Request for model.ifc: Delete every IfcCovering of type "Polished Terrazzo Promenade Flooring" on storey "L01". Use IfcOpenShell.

First a look at what the model holds.

```python
import ifcopenshell
import ifcopenshell.util.element

model = ifcopenshell.open("model.ifc")
print(model.schema)
storey = next(s for s in model.by_type("IfcBuildingStorey") if s.Name == "L01")
coverings = [e for e in ifcopenshell.util.element.get_decomposition(storey) if e.is_a("IfcCovering")]
seen = {}
for e in coverings:
    element_type = ifcopenshell.util.element.get_type(e)
    name = element_type.Name if element_type not in (None, e) else None
    seen[name] = seen.get(name, 0) + 1
for name, count in sorted(seen.items(), key=str):
    print(count, "x", name)
```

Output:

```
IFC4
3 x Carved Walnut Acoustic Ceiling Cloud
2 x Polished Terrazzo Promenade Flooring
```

```python
import ifcopenshell
import ifcopenshell.api.root
import ifcopenshell.util.element

model = ifcopenshell.open("model.ifc")

storey = next(s for s in model.by_type("IfcBuildingStorey") if s.Name == "L01")
coverings = [e for e in ifcopenshell.util.element.get_decomposition(storey) if e.is_a("IfcCovering")]
targets = [e for e in coverings if (t := ifcopenshell.util.element.get_type(e)) not in (None, e) and t.Name == "Polished Terrazzo Promenade Flooring"]

for e in targets:
    ifcopenshell.api.root.remove_product(model, product=e)
print(len(targets), "removed")

model.write("model_updated.ifc")
```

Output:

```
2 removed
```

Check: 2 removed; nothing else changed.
